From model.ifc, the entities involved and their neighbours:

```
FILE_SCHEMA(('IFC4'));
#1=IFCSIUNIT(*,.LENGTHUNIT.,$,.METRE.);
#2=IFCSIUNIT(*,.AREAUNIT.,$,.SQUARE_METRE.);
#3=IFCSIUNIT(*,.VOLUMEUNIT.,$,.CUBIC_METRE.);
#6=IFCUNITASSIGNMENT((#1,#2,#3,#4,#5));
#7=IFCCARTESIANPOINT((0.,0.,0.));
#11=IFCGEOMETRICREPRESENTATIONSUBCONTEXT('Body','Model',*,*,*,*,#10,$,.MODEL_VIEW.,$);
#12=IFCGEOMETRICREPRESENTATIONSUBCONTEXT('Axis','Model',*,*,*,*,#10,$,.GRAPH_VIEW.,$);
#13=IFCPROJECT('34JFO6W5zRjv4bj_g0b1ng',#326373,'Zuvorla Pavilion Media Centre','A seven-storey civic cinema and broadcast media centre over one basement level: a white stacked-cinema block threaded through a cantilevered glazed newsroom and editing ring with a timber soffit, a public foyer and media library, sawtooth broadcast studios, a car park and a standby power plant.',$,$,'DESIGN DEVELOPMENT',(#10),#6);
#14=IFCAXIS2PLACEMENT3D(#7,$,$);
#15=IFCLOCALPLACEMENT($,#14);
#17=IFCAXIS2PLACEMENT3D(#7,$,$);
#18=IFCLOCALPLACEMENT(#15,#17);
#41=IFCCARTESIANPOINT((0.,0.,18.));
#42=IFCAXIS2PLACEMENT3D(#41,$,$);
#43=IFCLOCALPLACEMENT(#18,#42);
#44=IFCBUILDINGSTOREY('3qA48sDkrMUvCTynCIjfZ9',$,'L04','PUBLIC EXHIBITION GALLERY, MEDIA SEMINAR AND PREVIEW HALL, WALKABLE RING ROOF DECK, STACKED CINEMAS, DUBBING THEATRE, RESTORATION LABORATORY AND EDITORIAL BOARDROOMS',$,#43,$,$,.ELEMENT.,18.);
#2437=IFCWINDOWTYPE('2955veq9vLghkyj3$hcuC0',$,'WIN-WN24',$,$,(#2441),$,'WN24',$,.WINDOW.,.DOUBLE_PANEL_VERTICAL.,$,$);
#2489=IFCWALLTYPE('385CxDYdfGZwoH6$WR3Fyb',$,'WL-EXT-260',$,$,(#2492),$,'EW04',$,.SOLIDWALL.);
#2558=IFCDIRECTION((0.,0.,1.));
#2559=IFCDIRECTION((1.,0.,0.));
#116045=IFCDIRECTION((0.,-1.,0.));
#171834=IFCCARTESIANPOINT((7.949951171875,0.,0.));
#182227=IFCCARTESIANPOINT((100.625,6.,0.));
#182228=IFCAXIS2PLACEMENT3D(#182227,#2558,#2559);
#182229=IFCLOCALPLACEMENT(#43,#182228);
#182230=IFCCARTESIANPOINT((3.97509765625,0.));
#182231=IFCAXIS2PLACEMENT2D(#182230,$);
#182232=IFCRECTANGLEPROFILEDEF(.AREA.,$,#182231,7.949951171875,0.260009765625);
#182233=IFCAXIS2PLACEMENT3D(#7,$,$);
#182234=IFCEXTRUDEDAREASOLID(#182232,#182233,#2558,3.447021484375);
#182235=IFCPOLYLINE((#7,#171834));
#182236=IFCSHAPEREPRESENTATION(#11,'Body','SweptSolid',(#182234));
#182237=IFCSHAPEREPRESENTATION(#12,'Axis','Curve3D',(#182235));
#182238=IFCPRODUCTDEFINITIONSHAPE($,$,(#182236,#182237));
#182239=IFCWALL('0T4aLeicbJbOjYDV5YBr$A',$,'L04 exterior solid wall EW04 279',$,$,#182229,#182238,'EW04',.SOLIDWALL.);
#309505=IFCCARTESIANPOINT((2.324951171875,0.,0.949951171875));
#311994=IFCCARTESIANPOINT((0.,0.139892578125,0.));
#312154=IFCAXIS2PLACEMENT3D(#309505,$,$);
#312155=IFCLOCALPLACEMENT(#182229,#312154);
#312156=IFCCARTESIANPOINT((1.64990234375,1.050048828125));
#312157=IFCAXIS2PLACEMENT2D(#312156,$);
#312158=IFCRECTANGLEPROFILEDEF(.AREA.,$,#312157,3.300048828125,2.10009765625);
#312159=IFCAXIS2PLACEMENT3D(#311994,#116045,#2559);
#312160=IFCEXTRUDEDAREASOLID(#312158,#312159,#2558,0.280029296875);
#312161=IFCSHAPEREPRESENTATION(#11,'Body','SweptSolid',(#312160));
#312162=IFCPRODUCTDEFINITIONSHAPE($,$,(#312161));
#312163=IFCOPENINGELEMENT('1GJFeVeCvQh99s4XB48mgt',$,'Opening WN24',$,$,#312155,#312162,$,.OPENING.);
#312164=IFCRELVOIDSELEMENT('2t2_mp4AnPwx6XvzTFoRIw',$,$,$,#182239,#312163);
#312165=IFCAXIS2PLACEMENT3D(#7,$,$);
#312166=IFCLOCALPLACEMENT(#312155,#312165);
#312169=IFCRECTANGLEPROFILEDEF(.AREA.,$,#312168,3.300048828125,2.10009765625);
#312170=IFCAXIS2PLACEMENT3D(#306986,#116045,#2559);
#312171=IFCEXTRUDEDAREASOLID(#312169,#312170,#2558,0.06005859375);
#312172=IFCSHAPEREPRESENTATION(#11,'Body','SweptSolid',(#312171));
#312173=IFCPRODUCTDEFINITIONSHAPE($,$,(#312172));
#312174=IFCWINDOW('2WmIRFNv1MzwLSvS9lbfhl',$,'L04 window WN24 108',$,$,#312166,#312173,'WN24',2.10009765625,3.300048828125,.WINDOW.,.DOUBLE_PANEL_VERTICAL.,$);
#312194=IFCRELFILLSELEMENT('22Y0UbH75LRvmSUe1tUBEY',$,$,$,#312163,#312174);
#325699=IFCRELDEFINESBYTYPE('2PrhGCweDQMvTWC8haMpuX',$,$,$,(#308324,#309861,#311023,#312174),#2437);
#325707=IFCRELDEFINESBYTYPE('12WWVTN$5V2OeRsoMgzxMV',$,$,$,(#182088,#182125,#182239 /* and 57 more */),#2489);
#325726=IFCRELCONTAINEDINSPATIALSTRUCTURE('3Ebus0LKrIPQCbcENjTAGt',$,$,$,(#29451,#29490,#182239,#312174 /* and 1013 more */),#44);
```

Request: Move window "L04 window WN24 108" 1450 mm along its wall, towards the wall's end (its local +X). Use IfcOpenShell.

```python
import ifcopenshell
import ifcopenshell.api.geometry
import ifcopenshell.util.placement
import ifcopenshell.util.unit

model = ifcopenshell.open("model.ifc")
unit_scale = ifcopenshell.util.unit.calculate_unit_scale(model)

window = model.by_guid("2WmIRFNv1MzwLSvS9lbfhl")
opening = window.FillsVoids[0].RelatingOpeningElement
wall = opening.VoidsElements[0].RelatingBuildingElement

wall_matrix = ifcopenshell.util.placement.get_local_placement(wall.ObjectPlacement)
shift = wall_matrix[:3, 0] * 1.45 / unit_scale
before = ifcopenshell.util.placement.get_local_placement(window.ObjectPlacement)[:3, 3].copy()

# The window is placed relative to its opening, so it follows when the opening moves.
matrix = ifcopenshell.util.placement.get_local_placement(opening.ObjectPlacement)
matrix[:3, 3] += shift
ifcopenshell.api.geometry.edit_object_placement(
    model, product=opening, matrix=matrix, is_si=False, should_transform_children=True
)

after = ifcopenshell.util.placement.get_local_placement(window.ObjectPlacement)[:3, 3]
print("window moved by", (after - before).round(3) + 0.0)

model.write("model_v2.ifc")
```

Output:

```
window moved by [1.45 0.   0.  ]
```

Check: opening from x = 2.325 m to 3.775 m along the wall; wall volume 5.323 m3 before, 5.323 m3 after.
